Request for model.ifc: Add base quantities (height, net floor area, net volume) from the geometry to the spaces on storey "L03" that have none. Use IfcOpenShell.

First a look at what the model holds.

```python
import ifcopenshell
import ifcopenshell.util.element
import ifcopenshell.util.unit

model = ifcopenshell.open("model.ifc")
print(model.schema)
for unit_type in ("LENGTHUNIT", "AREAUNIT", "VOLUMEUNIT"):
    print(unit_type, ifcopenshell.util.unit.calculate_unit_scale(model, unit_type))
storey = next(s for s in model.by_type("IfcBuildingStorey") if s.Name == "L03")
spaces = [e for e in ifcopenshell.util.element.get_decomposition(storey) if e.is_a("IfcSpace")]
for e in sorted(spaces, key=lambda e: e.id()):
    print(e.id(), e.is_a(), e.Name, list(ifcopenshell.util.element.get_psets(e, qtos_only=True)), sep=" | ")
```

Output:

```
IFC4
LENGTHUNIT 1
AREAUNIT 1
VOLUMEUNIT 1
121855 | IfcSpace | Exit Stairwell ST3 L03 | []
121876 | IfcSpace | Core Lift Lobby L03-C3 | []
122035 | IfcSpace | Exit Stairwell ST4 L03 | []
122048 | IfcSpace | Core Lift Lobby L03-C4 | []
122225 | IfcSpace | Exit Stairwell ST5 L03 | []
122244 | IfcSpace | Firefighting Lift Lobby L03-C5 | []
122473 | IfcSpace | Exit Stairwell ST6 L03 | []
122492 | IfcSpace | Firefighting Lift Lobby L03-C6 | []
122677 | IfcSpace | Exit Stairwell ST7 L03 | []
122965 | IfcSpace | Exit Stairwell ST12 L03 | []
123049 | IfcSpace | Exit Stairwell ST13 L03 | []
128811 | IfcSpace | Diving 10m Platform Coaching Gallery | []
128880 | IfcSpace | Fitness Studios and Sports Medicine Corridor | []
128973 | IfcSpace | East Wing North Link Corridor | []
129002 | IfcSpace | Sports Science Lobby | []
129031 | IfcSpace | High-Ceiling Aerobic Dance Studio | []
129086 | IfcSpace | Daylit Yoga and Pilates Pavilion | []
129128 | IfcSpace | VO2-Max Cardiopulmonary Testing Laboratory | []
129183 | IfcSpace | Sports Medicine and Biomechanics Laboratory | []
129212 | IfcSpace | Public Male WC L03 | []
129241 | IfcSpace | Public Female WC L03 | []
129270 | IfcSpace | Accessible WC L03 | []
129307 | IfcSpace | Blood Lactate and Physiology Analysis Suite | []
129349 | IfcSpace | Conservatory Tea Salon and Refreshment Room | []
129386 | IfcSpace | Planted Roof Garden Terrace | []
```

```python
import ifcopenshell
import ifcopenshell.api.pset
import ifcopenshell.geom
import ifcopenshell.util.element
import ifcopenshell.util.shape
import ifcopenshell.util.unit

model = ifcopenshell.open("model.ifc")
unit_scale = ifcopenshell.util.unit.calculate_unit_scale(model)
area_scale = ifcopenshell.util.unit.calculate_unit_scale(model, "AREAUNIT")
volume_scale = ifcopenshell.util.unit.calculate_unit_scale(model, "VOLUMEUNIT")
settings = ifcopenshell.geom.settings()

storey = next(s for s in model.by_type("IfcBuildingStorey") if s.Name == "L03")
spaces = [e for e in ifcopenshell.util.element.get_decomposition(storey) if e.is_a("IfcSpace")]

for e in sorted(spaces, key=lambda e: e.id()):
    if ifcopenshell.util.element.get_psets(e, qtos_only=True, should_inherit=False):
        continue
    # Geometry comes back in metres, in the element's own axes.
    shape = ifcopenshell.geom.create_shape(settings, e)
    values = {
        "Height": ifcopenshell.util.shape.get_z(shape.geometry) / unit_scale,
        "NetFloorArea": ifcopenshell.util.shape.get_footprint_area(shape.geometry) / area_scale,
        "NetVolume": ifcopenshell.util.shape.get_volume(shape.geometry) / volume_scale,
    }
    qto = ifcopenshell.api.pset.add_qto(model, product=e, name="Qto_SpaceBaseQuantities")
    ifcopenshell.api.pset.edit_qto(model, qto=qto, properties=values)
    print(e.id(), {k: round(v, 3) for k, v in values.items()})

model.write("model_rev.ifc")
```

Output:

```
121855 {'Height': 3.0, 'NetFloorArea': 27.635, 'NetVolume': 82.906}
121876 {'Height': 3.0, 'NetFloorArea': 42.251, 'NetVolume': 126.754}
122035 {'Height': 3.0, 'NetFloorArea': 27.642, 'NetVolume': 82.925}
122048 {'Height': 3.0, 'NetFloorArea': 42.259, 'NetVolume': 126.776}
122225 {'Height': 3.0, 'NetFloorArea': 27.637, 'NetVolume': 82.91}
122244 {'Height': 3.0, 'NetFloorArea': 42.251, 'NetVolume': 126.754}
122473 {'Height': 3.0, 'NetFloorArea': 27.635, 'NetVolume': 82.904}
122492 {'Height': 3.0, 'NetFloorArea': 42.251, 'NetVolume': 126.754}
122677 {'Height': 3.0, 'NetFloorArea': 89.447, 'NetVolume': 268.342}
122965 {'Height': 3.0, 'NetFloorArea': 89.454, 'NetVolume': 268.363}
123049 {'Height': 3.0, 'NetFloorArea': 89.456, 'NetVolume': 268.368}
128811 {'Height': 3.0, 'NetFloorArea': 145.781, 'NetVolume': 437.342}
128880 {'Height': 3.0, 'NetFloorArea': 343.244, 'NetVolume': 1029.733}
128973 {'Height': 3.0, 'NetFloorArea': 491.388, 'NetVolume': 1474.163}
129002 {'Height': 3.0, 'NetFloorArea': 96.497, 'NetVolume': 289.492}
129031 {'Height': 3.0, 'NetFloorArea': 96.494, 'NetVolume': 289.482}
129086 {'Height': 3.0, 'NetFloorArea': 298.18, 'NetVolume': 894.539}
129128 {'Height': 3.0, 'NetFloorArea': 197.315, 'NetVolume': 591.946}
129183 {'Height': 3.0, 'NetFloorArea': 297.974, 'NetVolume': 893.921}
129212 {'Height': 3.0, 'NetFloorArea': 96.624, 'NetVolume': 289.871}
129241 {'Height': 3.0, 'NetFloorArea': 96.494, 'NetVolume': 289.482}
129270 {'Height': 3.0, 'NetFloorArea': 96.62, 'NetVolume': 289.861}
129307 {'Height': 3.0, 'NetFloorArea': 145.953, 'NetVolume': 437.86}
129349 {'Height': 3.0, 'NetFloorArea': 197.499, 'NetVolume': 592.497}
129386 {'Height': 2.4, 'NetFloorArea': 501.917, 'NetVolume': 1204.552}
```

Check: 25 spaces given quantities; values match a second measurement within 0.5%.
